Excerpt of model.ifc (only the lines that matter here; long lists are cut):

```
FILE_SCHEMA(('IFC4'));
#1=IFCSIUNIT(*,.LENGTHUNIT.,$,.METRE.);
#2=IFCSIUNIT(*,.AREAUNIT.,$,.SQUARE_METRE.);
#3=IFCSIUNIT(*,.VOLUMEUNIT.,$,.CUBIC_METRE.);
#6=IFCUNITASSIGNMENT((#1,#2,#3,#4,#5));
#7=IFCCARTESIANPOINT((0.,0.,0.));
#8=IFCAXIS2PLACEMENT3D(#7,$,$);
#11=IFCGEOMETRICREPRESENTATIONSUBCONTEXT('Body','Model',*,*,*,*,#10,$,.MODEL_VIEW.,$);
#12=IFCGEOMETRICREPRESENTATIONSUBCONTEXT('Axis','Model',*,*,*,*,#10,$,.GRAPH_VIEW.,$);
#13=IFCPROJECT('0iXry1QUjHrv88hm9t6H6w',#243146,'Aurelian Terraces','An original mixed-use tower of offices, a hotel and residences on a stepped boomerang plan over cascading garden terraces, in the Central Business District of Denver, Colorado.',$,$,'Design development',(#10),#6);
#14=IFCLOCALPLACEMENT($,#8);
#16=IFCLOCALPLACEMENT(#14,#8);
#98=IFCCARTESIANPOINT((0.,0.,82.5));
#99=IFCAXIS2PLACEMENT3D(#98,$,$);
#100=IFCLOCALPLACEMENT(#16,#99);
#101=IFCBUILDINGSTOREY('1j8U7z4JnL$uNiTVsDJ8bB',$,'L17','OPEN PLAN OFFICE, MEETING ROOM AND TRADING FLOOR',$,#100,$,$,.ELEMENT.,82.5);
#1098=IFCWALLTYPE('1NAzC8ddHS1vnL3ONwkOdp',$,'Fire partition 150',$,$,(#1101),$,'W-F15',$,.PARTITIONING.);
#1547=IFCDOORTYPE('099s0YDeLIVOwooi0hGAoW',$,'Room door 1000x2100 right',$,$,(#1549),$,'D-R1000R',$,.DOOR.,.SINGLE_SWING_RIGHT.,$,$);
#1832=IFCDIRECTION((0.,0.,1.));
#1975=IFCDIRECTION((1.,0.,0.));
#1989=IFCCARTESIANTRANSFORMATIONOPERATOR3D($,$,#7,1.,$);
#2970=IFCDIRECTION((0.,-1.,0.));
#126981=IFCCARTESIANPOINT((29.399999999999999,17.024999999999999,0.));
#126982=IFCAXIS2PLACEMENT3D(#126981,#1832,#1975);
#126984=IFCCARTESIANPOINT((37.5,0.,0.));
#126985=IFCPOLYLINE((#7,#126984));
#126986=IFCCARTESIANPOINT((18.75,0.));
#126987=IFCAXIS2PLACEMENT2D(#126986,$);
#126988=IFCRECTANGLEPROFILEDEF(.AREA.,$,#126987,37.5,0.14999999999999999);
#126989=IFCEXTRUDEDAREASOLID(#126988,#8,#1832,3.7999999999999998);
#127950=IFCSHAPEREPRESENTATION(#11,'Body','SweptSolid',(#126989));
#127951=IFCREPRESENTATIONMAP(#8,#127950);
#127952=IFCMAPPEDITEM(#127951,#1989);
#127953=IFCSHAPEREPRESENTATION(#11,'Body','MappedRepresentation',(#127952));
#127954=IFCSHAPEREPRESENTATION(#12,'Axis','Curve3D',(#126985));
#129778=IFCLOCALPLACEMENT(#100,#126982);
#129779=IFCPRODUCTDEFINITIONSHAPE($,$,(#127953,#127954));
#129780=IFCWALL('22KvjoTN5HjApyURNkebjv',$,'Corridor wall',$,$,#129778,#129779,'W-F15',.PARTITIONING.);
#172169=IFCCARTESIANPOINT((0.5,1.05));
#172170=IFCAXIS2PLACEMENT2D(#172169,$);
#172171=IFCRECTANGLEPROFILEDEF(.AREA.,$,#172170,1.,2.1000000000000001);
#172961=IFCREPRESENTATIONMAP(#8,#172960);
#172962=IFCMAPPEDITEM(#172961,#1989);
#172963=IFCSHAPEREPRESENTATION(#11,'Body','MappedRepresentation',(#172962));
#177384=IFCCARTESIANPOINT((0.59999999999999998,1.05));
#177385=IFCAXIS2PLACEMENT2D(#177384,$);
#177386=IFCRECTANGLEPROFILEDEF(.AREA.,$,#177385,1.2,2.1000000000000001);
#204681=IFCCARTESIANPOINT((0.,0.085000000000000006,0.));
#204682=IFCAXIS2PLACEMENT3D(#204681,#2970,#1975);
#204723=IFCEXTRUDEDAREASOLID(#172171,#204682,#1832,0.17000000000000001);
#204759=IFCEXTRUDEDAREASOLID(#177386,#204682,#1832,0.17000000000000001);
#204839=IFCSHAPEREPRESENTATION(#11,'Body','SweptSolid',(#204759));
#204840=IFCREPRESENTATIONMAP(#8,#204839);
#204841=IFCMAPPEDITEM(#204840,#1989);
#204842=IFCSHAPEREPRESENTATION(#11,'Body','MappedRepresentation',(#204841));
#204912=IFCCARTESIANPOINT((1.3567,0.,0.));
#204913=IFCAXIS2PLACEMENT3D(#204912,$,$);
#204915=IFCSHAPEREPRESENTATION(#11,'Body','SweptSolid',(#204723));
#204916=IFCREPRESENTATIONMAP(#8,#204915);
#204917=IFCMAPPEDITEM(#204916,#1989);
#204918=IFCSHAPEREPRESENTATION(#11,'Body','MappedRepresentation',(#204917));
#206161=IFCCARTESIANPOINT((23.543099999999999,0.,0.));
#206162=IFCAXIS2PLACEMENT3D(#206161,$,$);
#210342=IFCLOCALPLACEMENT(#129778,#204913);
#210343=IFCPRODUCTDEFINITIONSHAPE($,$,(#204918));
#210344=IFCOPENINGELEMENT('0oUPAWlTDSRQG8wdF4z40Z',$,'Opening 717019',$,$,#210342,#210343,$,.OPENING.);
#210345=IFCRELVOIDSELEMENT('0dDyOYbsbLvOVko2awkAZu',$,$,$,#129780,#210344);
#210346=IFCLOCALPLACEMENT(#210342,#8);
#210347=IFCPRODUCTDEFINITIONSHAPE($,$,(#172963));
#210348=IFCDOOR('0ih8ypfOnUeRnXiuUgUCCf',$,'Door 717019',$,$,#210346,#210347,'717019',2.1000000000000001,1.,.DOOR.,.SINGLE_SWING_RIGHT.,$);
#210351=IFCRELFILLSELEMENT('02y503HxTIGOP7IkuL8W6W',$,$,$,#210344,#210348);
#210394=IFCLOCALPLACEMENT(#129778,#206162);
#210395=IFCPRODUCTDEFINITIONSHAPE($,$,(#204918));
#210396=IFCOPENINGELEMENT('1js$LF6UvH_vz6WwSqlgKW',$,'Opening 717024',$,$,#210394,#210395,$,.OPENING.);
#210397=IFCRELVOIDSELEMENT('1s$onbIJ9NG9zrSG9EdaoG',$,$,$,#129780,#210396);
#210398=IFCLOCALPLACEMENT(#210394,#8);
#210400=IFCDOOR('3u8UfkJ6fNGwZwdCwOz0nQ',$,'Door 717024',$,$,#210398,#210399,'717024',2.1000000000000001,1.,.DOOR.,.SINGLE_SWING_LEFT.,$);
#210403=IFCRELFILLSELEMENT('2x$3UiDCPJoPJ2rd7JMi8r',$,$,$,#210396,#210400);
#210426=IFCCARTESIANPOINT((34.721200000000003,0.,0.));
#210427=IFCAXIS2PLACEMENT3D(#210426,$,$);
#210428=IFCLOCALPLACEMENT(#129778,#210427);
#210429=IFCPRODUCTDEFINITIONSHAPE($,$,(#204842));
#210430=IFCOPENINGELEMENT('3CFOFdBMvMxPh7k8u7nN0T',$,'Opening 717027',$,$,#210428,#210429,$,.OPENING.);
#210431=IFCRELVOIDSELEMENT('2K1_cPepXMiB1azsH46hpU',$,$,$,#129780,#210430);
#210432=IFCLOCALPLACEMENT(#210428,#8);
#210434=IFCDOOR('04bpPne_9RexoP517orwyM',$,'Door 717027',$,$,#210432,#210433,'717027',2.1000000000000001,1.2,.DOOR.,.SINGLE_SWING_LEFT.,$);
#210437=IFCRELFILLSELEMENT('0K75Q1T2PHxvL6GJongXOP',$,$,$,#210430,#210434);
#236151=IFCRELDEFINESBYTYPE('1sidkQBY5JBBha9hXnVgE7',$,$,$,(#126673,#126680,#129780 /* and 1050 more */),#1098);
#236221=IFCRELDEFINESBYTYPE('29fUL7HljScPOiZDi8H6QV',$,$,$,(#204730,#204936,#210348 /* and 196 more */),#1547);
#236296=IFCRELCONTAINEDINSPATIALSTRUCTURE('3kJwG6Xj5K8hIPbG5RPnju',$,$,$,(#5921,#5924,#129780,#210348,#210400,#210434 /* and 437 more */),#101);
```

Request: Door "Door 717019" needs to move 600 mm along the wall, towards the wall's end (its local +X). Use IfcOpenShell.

```python
import ifcopenshell
import ifcopenshell.api.geometry
import ifcopenshell.util.placement
import ifcopenshell.util.unit

model = ifcopenshell.open("model.ifc")
unit_scale = ifcopenshell.util.unit.calculate_unit_scale(model)

door = model.by_guid("0ih8ypfOnUeRnXiuUgUCCf")
opening = door.FillsVoids[0].RelatingOpeningElement
wall = opening.VoidsElements[0].RelatingBuildingElement

wall_matrix = ifcopenshell.util.placement.get_local_placement(wall.ObjectPlacement)
shift = wall_matrix[:3, 0] * 0.6 / unit_scale
before = ifcopenshell.util.placement.get_local_placement(door.ObjectPlacement)[:3, 3].copy()

# The door is placed relative to its opening, so it follows when the opening moves.
matrix = ifcopenshell.util.placement.get_local_placement(opening.ObjectPlacement)
matrix[:3, 3] += shift
ifcopenshell.api.geometry.edit_object_placement(
    model, product=opening, matrix=matrix, is_si=False, should_transform_children=True
)

after = ifcopenshell.util.placement.get_local_placement(door.ObjectPlacement)[:3, 3]
print("door moved by", (after - before).round(3) + 0.0)

model.write("model-out.ifc")
```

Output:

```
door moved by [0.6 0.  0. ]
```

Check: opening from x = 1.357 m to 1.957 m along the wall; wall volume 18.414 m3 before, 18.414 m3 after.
